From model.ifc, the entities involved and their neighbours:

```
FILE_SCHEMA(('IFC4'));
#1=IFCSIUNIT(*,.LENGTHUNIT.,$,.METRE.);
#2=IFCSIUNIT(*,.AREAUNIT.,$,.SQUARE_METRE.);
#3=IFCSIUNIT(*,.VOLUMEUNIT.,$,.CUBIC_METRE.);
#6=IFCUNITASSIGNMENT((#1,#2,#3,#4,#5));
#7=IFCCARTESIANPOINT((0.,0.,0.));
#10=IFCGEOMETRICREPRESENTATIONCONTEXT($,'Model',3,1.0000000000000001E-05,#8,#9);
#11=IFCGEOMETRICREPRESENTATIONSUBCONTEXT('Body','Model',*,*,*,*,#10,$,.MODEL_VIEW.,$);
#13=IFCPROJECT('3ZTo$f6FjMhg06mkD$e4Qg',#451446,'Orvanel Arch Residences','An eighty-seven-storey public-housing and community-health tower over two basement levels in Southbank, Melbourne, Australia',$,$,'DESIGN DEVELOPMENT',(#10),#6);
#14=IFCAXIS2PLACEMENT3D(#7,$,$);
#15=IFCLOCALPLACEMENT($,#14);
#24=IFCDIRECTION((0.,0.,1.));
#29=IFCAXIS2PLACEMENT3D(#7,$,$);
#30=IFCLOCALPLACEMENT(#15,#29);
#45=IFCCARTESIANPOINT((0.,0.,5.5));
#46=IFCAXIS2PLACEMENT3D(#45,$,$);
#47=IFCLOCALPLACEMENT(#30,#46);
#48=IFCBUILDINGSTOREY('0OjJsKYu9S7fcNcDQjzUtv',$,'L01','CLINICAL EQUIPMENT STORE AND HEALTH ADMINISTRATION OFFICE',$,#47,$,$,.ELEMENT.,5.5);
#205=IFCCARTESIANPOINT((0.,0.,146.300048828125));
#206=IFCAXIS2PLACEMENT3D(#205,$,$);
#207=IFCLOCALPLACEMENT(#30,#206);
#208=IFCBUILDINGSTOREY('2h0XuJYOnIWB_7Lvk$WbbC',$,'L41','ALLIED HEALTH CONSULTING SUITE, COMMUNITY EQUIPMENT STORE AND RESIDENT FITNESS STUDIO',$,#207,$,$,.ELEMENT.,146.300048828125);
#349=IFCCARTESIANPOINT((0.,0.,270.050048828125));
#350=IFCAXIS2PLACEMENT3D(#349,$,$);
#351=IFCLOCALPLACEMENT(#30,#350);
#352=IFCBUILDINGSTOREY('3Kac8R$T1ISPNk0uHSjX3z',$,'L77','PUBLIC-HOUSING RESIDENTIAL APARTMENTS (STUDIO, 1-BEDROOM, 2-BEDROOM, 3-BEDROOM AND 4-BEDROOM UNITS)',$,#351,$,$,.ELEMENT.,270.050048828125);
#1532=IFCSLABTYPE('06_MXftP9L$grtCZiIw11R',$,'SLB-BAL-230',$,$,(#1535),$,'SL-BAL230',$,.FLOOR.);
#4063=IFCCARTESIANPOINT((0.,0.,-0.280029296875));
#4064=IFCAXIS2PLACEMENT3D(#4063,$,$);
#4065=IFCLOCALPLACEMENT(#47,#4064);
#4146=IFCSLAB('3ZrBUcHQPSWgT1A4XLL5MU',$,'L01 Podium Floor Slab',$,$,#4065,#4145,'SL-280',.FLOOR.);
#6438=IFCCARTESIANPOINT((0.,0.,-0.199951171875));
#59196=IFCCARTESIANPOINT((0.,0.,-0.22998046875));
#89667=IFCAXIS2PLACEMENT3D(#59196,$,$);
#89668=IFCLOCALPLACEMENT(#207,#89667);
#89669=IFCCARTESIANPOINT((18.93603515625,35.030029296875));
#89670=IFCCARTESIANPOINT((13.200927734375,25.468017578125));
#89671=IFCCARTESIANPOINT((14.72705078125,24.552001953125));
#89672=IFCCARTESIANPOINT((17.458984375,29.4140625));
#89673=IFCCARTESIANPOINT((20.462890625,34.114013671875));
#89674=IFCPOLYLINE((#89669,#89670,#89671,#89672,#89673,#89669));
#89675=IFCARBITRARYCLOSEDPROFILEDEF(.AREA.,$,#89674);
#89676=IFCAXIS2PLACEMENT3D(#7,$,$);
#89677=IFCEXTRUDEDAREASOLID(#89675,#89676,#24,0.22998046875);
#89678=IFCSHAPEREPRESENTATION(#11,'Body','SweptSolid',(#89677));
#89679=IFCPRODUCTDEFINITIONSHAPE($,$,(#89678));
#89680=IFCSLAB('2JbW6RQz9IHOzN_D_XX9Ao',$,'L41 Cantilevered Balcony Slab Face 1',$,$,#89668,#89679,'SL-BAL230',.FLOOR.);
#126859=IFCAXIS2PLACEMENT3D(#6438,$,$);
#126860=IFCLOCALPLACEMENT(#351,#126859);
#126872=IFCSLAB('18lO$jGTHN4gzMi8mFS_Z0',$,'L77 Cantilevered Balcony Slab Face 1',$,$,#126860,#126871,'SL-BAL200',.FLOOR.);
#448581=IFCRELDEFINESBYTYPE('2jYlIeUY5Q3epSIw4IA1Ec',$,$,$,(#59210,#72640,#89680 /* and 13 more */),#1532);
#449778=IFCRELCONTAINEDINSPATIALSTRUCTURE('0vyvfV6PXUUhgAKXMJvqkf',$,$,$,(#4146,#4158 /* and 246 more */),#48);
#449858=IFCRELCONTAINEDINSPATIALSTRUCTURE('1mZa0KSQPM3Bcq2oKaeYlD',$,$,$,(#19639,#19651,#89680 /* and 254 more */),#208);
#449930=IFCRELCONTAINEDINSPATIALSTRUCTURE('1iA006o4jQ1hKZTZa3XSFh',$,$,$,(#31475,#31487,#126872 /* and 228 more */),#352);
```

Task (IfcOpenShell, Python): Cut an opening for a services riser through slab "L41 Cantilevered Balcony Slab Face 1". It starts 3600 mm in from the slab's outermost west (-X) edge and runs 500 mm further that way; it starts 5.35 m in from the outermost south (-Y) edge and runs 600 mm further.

```python
import numpy as np
import ifcopenshell
import ifcopenshell.api.feature
import ifcopenshell.api.geometry
import ifcopenshell.api.root
import ifcopenshell.geom
import ifcopenshell.util.placement
import ifcopenshell.util.representation
import ifcopenshell.util.shape
import ifcopenshell.util.unit

model = ifcopenshell.open("model.ifc")
unit_scale = ifcopenshell.util.unit.calculate_unit_scale(model)
settings = ifcopenshell.geom.settings()


def volume(element):
    """Net volume in cubic metres, openings subtracted."""
    shape = ifcopenshell.geom.create_shape(settings, element)
    return ifcopenshell.util.shape.get_volume(shape.geometry)


slab = model.by_guid("2JbW6RQz9IHOzN_D_XX9Ao")
before = volume(slab)

# Extent in the slab's own axes, in metres. The edges named are its -X and -Y sides.
slab_shape = ifcopenshell.geom.create_shape(settings, slab)
vertices = ifcopenshell.util.shape.get_vertices(slab_shape.geometry)
x_min, y_min, bottom = vertices.min(axis=0)
top = vertices[:, 2].max()

opening = ifcopenshell.api.root.create_entity(model, ifc_class="IfcOpeningElement", name="Services riser opening", predefined_type="OPENING")
context = ifcopenshell.util.representation.get_context(model, "Model", "Body", "MODEL_VIEW")
width, depth = 0.5, 0.6
outline = [(0.0, 0.0), (width, 0.0), (width, depth), (0.0, depth), (0.0, 0.0)]
# Overshoot both faces by 50 mm so the cut is clean.
shape = ifcopenshell.api.geometry.add_slab_representation(
    model, context=context, depth=top - bottom + 0.1, polyline=outline
)
ifcopenshell.api.geometry.assign_representation(model, product=opening, representation=shape)

matrix = ifcopenshell.util.placement.get_local_placement(slab.ObjectPlacement)
matrix[:, 3] = matrix @ np.append(np.array([x_min + 3.6, y_min + 5.35, bottom - 0.05]) / unit_scale, 1.0)
ifcopenshell.api.geometry.edit_object_placement(model, product=opening, matrix=matrix, is_si=False)
ifcopenshell.api.feature.add_feature(model, feature=opening, element=slab)

after = volume(slab)

print(f"slab volume {before:.3f} -> {after:.3f} m3")

model.write("model-out.ifc")
```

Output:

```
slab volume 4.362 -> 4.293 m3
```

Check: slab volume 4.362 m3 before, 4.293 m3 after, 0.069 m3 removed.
